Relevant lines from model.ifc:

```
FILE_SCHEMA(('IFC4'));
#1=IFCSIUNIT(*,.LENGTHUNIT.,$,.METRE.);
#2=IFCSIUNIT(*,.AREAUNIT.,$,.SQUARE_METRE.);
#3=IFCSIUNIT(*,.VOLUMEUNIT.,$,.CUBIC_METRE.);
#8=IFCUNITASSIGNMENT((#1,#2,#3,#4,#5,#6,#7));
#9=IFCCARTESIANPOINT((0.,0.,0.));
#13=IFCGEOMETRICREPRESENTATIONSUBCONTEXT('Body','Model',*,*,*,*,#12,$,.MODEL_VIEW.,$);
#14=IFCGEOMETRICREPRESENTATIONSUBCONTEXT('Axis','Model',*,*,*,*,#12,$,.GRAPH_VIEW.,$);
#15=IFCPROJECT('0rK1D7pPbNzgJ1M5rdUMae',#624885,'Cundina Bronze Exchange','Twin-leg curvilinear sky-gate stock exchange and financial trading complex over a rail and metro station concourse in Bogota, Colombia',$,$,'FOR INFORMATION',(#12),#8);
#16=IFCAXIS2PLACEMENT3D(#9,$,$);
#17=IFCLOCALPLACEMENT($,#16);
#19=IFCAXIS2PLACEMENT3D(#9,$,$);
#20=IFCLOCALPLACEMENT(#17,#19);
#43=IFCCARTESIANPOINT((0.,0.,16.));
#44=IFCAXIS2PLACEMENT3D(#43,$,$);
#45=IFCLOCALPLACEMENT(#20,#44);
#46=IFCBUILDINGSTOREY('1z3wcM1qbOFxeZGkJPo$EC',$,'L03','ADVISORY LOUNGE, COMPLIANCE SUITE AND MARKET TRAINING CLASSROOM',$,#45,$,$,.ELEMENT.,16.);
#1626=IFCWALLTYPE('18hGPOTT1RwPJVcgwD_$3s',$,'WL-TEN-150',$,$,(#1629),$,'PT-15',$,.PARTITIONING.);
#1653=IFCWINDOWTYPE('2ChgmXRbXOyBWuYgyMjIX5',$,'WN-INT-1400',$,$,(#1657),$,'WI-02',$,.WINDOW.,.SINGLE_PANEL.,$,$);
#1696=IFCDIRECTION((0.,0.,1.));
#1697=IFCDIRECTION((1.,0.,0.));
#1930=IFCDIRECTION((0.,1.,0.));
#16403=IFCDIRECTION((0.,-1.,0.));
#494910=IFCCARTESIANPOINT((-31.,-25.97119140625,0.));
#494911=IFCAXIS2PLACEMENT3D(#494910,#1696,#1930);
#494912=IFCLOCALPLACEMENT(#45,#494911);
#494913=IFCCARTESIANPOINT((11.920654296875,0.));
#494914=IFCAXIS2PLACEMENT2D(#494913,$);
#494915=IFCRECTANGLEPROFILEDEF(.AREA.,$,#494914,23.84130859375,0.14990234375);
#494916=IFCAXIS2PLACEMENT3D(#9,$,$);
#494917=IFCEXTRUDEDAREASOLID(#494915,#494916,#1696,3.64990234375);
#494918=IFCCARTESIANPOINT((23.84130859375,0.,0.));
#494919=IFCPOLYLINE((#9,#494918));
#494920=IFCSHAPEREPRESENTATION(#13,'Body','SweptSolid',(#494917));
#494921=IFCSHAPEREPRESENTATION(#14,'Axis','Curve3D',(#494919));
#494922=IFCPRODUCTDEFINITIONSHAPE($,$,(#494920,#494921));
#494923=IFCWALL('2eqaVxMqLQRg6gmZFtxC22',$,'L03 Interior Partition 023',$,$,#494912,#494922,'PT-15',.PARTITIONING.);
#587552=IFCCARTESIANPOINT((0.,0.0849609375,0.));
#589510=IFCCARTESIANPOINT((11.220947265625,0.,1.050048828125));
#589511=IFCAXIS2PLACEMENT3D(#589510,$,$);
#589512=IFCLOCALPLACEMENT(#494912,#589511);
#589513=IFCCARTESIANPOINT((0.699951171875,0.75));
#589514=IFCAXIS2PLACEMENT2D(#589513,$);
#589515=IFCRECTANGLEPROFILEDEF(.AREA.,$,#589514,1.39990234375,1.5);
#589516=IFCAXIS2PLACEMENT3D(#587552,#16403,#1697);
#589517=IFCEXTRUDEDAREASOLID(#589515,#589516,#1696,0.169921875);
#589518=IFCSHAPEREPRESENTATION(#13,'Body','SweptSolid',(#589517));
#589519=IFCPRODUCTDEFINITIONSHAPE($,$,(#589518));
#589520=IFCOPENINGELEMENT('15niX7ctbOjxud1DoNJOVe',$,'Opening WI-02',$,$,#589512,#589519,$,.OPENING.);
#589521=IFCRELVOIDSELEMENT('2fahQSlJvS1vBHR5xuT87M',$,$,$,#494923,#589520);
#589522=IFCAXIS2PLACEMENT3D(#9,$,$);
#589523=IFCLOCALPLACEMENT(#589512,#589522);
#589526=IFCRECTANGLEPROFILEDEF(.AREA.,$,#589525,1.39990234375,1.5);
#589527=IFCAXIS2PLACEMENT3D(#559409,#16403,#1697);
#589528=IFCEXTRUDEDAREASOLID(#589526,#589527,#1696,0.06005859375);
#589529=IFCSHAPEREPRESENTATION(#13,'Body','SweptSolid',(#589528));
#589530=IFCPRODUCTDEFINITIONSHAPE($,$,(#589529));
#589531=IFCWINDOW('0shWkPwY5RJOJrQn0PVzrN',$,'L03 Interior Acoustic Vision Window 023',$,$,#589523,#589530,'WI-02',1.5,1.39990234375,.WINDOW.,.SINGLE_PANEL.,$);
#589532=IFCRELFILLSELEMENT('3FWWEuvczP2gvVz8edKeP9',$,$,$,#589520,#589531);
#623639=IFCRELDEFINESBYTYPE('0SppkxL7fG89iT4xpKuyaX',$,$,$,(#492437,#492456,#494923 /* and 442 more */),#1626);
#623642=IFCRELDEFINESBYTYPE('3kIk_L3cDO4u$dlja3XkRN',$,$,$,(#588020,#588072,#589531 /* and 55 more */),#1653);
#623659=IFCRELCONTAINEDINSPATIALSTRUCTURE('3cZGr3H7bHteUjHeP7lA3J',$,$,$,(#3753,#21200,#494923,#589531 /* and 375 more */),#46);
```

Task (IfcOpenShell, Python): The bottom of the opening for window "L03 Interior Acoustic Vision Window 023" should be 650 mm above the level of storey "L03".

```python
import numpy as np
import ifcopenshell
import ifcopenshell.api.geometry
import ifcopenshell.geom
import ifcopenshell.util.element
import ifcopenshell.util.placement
import ifcopenshell.util.shape
import ifcopenshell.util.unit

model = ifcopenshell.open("model.ifc")
unit_scale = ifcopenshell.util.unit.calculate_unit_scale(model)

window = model.by_id(589531)
opening = window.FillsVoids[0].RelatingOpeningElement
storey = ifcopenshell.util.element.get_container(window, ifc_class="IfcBuildingStorey")
level = ifcopenshell.util.placement.get_local_placement(storey.ObjectPlacement)[2, 3]

# The opening's origin need not be at the sill, so measure its lowest point.
shape = ifcopenshell.geom.create_shape(ifcopenshell.geom.settings(), opening)
bottom = ifcopenshell.util.shape.get_shape_bottom_elevation(shape, shape.geometry) / unit_scale
dz = level + 0.65 - bottom

shift = np.array([0.0, 0.0, dz])
# The window is placed relative to its opening, so it follows when the opening moves.
matrix = ifcopenshell.util.placement.get_local_placement(opening.ObjectPlacement)
matrix[:3, 3] += shift
ifcopenshell.api.geometry.edit_object_placement(
    model, product=opening, matrix=matrix, is_si=False, should_transform_children=True
)

print(f"moved by {dz * unit_scale:+.3f} m")

model.write("model_edited.ifc")
```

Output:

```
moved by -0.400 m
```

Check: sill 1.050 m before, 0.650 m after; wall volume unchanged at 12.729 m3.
